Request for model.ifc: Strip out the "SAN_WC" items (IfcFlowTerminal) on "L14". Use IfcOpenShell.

First a look at what the model holds.

```python
import ifcopenshell
import ifcopenshell.util.element

model = ifcopenshell.open("model.ifc")
print(model.schema)
storey = next(s for s in model.by_type("IfcBuildingStorey") if s.Name == "L14")
terminals = [e for e in ifcopenshell.util.element.get_decomposition(storey) if e.is_a("IfcFlowTerminal")]
seen = {}
for e in terminals:
    element_type = ifcopenshell.util.element.get_type(e)
    name = element_type.Name if element_type not in (None, e) else None
    seen[name] = seen.get(name, 0) + 1
for name, count in sorted(seen.items(), key=str):
    print(count, "x", name)
```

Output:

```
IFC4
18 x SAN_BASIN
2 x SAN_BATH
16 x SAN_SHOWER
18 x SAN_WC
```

```python
import ifcopenshell
import ifcopenshell.api.root
import ifcopenshell.util.element

model = ifcopenshell.open("model.ifc")

storey = next(s for s in model.by_type("IfcBuildingStorey") if s.Name == "L14")
terminals = [e for e in ifcopenshell.util.element.get_decomposition(storey) if e.is_a("IfcFlowTerminal")]
targets = [e for e in terminals if (t := ifcopenshell.util.element.get_type(e)) not in (None, e) and t.Name == "SAN_WC"]

for e in targets:
    ifcopenshell.api.root.remove_product(model, product=e)
print(len(targets), "removed")

model.write("model_rev.ifc")
```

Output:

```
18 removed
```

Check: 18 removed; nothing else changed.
